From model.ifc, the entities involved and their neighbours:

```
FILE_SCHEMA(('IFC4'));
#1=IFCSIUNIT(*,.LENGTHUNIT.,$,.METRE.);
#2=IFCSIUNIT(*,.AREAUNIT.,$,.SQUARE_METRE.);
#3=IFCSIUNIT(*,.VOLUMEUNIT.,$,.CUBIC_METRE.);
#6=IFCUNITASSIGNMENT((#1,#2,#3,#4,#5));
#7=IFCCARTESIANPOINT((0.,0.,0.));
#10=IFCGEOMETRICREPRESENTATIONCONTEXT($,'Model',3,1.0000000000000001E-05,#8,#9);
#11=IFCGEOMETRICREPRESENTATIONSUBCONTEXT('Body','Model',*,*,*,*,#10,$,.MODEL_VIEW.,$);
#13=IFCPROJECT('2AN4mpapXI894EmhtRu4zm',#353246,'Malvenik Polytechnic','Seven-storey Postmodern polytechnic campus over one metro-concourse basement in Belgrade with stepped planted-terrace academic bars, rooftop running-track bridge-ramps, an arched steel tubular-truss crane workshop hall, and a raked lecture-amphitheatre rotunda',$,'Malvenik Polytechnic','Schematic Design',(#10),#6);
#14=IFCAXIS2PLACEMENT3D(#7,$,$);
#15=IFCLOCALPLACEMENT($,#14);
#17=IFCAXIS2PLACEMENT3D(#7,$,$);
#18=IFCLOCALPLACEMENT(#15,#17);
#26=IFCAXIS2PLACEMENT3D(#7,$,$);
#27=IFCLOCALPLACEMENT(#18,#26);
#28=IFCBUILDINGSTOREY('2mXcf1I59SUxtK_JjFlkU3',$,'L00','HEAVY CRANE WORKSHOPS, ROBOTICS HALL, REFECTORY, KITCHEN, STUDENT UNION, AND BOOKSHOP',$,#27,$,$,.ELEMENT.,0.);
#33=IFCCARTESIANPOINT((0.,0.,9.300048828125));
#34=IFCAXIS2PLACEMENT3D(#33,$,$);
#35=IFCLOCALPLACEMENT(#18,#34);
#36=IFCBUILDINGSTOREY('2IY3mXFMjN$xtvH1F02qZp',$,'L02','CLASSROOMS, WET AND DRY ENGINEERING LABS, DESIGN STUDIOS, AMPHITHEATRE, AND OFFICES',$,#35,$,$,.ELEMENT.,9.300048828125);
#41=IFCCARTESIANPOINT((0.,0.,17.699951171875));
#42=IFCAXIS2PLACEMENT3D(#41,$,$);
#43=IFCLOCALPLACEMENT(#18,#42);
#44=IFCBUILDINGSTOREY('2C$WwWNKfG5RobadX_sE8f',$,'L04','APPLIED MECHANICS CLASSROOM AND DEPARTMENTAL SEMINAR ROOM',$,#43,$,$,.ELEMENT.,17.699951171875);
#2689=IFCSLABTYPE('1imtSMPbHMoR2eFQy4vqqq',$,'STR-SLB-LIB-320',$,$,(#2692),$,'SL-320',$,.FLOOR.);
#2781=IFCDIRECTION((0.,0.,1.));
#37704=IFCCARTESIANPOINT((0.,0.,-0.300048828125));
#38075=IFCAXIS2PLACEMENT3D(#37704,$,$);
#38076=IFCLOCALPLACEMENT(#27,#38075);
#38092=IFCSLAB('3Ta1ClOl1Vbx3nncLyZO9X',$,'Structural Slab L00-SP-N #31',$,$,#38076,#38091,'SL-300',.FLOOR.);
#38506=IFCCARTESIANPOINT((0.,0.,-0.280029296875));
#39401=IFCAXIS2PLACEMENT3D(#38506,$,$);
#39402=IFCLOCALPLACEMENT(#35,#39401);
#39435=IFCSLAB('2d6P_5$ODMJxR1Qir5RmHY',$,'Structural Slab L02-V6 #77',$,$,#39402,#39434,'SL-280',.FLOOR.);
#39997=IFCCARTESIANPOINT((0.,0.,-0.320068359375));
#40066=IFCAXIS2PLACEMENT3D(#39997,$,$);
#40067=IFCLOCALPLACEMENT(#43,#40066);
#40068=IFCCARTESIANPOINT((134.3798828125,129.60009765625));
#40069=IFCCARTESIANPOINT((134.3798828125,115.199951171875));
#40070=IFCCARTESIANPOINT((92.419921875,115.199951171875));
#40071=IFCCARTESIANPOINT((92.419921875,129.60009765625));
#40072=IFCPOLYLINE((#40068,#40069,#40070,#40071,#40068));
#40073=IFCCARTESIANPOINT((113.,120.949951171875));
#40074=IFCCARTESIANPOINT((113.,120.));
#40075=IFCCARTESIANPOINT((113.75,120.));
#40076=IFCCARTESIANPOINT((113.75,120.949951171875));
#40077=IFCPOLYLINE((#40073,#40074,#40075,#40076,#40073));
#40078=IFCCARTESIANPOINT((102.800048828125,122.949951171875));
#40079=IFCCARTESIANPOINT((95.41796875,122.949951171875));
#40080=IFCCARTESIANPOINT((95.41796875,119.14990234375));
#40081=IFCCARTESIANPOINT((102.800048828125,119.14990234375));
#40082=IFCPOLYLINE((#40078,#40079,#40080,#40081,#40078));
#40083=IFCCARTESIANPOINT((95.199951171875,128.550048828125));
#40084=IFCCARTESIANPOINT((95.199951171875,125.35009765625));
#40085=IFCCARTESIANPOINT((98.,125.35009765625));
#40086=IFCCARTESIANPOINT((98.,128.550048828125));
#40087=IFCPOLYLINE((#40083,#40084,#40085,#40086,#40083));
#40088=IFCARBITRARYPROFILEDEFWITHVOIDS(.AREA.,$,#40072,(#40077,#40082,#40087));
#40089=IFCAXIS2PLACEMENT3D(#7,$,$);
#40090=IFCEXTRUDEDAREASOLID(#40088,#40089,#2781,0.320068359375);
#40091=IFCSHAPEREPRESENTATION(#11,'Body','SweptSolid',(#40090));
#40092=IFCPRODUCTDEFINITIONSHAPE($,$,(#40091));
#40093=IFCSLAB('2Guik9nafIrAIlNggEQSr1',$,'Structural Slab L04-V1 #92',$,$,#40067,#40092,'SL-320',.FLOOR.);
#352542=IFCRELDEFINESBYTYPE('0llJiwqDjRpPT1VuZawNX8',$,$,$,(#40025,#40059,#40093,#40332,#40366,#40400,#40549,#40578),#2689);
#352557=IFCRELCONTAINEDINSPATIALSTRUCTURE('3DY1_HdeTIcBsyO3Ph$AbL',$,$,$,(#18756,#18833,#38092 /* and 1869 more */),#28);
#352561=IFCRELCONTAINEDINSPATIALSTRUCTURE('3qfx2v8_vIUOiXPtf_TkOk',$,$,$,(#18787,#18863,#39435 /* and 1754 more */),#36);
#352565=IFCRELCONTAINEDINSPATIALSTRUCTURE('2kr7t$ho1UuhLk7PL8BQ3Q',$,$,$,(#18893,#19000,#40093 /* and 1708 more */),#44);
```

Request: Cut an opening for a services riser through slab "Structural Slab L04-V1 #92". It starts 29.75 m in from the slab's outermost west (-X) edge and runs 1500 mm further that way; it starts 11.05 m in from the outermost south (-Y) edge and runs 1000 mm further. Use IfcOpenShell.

```python
import numpy as np
import ifcopenshell
import ifcopenshell.api.feature
import ifcopenshell.api.geometry
import ifcopenshell.api.root
import ifcopenshell.geom
import ifcopenshell.util.placement
import ifcopenshell.util.representation
import ifcopenshell.util.shape
import ifcopenshell.util.unit

model = ifcopenshell.open("model.ifc")
unit_scale = ifcopenshell.util.unit.calculate_unit_scale(model)
settings = ifcopenshell.geom.settings()


def volume(element):
    """Net volume in cubic metres, openings subtracted."""
    shape = ifcopenshell.geom.create_shape(settings, element)
    return ifcopenshell.util.shape.get_volume(shape.geometry)


slab = model.by_guid("2Guik9nafIrAIlNggEQSr1")
before = volume(slab)

# Extent in the slab's own axes, in metres. The edges named are its -X and -Y sides.
slab_shape = ifcopenshell.geom.create_shape(settings, slab)
vertices = ifcopenshell.util.shape.get_vertices(slab_shape.geometry)
x_min, y_min, bottom = vertices.min(axis=0)
top = vertices[:, 2].max()

opening = ifcopenshell.api.root.create_entity(model, ifc_class="IfcOpeningElement", name="Services riser opening", predefined_type="OPENING")
context = ifcopenshell.util.representation.get_context(model, "Model", "Body", "MODEL_VIEW")
width, depth = 1.5, 1
outline = [(0.0, 0.0), (width, 0.0), (width, depth), (0.0, depth), (0.0, 0.0)]
# Overshoot both faces by 50 mm so the cut is clean.
shape = ifcopenshell.api.geometry.add_slab_representation(
    model, context=context, depth=top - bottom + 0.1, polyline=outline
)
ifcopenshell.api.geometry.assign_representation(model, product=opening, representation=shape)

matrix = ifcopenshell.util.placement.get_local_placement(slab.ObjectPlacement)
matrix[:, 3] = matrix @ np.append(np.array([x_min + 29.75, y_min + 11.05, bottom - 0.05]) / unit_scale, 1.0)
ifcopenshell.api.geometry.edit_object_placement(model, product=opening, matrix=matrix, is_si=False)
ifcopenshell.api.feature.add_feature(model, feature=opening, element=slab)

after = volume(slab)

print(f"slab volume {before:.3f} -> {after:.3f} m3")

model.write("model-out.ifc")
```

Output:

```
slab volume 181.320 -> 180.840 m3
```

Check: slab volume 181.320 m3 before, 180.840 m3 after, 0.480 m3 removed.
